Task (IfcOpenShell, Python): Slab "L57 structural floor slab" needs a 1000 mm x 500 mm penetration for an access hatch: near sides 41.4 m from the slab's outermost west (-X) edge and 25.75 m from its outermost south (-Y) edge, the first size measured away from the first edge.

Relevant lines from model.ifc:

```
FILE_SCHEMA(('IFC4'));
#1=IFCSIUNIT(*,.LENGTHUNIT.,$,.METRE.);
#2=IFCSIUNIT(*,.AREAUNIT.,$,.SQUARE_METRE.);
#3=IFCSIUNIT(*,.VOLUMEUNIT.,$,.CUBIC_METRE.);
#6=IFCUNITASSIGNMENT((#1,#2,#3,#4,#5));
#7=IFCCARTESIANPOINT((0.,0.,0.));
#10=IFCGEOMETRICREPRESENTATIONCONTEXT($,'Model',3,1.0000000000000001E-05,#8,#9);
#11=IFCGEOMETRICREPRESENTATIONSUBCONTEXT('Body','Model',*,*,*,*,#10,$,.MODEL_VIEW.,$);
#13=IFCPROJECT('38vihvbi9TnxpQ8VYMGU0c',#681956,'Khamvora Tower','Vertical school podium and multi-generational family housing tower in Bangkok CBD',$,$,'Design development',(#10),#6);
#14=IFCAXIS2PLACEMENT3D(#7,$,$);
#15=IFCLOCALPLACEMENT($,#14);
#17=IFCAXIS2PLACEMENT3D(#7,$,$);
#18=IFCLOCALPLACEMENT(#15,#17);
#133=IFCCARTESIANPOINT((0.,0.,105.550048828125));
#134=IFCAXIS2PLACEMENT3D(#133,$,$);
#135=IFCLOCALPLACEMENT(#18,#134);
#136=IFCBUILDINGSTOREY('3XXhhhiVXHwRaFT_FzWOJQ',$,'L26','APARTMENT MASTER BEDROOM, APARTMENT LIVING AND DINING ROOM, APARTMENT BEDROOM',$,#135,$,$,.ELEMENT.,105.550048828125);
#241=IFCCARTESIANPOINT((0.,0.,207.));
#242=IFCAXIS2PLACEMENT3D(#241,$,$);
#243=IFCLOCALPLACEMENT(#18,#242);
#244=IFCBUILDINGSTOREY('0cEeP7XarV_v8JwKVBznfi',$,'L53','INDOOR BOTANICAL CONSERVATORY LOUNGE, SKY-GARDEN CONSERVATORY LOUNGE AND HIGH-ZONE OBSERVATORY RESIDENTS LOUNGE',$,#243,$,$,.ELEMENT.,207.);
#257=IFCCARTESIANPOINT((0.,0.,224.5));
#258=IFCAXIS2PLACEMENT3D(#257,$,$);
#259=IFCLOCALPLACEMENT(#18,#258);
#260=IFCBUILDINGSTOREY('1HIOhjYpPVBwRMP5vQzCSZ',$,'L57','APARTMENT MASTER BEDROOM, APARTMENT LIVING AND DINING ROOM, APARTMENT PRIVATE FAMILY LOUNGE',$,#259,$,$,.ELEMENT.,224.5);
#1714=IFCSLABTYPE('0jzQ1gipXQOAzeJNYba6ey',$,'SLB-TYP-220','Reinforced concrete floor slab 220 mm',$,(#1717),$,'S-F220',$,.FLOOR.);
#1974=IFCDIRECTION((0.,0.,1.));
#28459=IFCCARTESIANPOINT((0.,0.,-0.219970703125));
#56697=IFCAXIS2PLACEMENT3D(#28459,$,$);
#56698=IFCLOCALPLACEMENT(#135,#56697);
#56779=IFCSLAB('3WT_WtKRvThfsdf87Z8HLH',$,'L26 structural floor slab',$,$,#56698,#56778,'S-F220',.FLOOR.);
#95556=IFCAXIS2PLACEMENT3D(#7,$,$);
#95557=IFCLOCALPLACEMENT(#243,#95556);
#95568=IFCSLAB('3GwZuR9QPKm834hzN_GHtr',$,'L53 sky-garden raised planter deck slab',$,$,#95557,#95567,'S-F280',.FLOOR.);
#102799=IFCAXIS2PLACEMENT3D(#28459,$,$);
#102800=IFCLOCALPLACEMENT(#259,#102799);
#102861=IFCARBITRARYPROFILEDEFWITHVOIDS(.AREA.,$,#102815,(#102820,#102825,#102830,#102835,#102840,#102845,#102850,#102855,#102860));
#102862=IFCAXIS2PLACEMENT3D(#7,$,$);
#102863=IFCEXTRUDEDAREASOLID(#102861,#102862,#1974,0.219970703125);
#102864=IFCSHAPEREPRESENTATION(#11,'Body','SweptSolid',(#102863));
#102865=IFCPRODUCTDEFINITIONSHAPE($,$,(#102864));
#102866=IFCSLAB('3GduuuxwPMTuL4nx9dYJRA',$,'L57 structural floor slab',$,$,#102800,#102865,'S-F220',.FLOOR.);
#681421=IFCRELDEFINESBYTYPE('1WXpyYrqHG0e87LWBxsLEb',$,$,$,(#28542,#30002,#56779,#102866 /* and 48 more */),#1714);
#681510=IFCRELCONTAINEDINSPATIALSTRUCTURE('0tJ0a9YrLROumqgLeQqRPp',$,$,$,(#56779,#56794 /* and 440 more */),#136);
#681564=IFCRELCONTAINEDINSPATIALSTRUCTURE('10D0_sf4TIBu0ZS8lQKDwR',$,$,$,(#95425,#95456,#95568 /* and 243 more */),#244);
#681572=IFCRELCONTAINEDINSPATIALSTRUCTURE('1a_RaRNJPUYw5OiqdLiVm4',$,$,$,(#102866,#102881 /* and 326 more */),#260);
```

```python
import numpy as np
import ifcopenshell
import ifcopenshell.api.feature
import ifcopenshell.api.geometry
import ifcopenshell.api.root
import ifcopenshell.geom
import ifcopenshell.util.placement
import ifcopenshell.util.representation
import ifcopenshell.util.shape
import ifcopenshell.util.unit

model = ifcopenshell.open("model.ifc")
unit_scale = ifcopenshell.util.unit.calculate_unit_scale(model)
settings = ifcopenshell.geom.settings()


def volume(element):
    """Net volume in cubic metres, openings subtracted."""
    shape = ifcopenshell.geom.create_shape(settings, element)
    return ifcopenshell.util.shape.get_volume(shape.geometry)


slab = model.by_guid("3GduuuxwPMTuL4nx9dYJRA")
before = volume(slab)

# Extent in the slab's own axes, in metres. The edges named are its -X and -Y sides.
slab_shape = ifcopenshell.geom.create_shape(settings, slab)
vertices = ifcopenshell.util.shape.get_vertices(slab_shape.geometry)
x_min, y_min, bottom = vertices.min(axis=0)
top = vertices[:, 2].max()

opening = ifcopenshell.api.root.create_entity(model, ifc_class="IfcOpeningElement", name="Access hatch opening", predefined_type="OPENING")
context = ifcopenshell.util.representation.get_context(model, "Model", "Body", "MODEL_VIEW")
width, depth = 1, 0.5
outline = [(0.0, 0.0), (width, 0.0), (width, depth), (0.0, depth), (0.0, 0.0)]
# Overshoot both faces by 50 mm so the cut is clean.
shape = ifcopenshell.api.geometry.add_slab_representation(
    model, context=context, depth=top - bottom + 0.1, polyline=outline
)
ifcopenshell.api.geometry.assign_representation(model, product=opening, representation=shape)

matrix = ifcopenshell.util.placement.get_local_placement(slab.ObjectPlacement)
matrix[:, 3] = matrix @ np.append(np.array([x_min + 41.4, y_min + 25.75, bottom - 0.05]) / unit_scale, 1.0)
ifcopenshell.api.geometry.edit_object_placement(model, product=opening, matrix=matrix, is_si=False)
ifcopenshell.api.feature.add_feature(model, feature=opening, element=slab)

after = volume(slab)

print(f"slab volume {before:.3f} -> {after:.3f} m3")

model.write("model-out.ifc")
```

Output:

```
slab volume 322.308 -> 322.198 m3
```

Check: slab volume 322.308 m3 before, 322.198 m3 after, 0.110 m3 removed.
